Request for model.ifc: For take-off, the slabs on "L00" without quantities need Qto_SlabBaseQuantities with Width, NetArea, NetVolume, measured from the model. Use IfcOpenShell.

First a look at what the model holds.

```python
import ifcopenshell
import ifcopenshell.util.element
import ifcopenshell.util.unit

model = ifcopenshell.open("model.ifc")
print(model.schema)
for unit_type in ("LENGTHUNIT", "AREAUNIT", "VOLUMEUNIT"):
    print(unit_type, ifcopenshell.util.unit.calculate_unit_scale(model, unit_type))
storey = next(s for s in model.by_type("IfcBuildingStorey") if s.Name == "L00")
slabs = [e for e in ifcopenshell.util.element.get_decomposition(storey) if e.is_a("IfcSlab")]
for e in sorted(slabs, key=lambda e: e.id()):
    print(e.id(), e.is_a(), e.Name, list(ifcopenshell.util.element.get_psets(e, qtos_only=True)), sep=" | ")
```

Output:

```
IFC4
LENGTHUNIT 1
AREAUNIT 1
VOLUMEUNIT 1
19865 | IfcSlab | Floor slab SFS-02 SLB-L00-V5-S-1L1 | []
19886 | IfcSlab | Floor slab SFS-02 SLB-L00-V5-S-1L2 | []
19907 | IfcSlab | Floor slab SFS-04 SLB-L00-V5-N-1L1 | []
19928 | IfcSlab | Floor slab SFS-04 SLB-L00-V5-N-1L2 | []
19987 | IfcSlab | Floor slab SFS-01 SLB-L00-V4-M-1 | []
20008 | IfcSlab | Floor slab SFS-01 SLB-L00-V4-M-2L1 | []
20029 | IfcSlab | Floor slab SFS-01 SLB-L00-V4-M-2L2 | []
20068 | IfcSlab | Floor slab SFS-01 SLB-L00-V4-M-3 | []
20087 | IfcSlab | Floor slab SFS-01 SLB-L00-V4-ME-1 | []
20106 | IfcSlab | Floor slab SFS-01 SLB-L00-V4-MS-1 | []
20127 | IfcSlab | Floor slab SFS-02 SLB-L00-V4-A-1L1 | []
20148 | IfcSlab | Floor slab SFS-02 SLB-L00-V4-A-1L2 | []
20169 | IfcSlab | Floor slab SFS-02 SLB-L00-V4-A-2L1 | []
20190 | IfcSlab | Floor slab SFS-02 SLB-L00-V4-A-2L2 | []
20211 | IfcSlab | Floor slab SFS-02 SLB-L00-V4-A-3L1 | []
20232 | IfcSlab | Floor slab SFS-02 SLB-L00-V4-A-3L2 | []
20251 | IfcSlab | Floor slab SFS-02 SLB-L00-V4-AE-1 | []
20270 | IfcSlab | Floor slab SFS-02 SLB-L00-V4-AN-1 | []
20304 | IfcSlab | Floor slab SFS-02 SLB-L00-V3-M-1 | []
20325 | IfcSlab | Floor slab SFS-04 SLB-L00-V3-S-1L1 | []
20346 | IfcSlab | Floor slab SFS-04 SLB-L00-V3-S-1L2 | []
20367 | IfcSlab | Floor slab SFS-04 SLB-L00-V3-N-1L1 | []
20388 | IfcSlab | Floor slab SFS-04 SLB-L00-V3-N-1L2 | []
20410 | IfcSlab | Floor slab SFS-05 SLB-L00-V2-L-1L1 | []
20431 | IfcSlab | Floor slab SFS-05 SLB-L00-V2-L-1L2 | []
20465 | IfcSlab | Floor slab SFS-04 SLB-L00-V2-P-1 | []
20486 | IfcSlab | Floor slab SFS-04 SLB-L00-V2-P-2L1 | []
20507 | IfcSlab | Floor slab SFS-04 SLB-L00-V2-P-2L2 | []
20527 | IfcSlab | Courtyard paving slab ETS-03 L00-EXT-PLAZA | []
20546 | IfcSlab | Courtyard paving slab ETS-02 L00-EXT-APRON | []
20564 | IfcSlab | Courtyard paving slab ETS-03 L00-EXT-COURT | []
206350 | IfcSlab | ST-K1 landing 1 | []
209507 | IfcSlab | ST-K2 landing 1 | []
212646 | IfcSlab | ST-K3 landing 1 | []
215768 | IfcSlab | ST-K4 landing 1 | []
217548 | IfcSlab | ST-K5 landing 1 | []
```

```python
import ifcopenshell
import ifcopenshell.api.pset
import ifcopenshell.geom
import ifcopenshell.util.element
import ifcopenshell.util.shape
import ifcopenshell.util.unit

model = ifcopenshell.open("model.ifc")
unit_scale = ifcopenshell.util.unit.calculate_unit_scale(model)
area_scale = ifcopenshell.util.unit.calculate_unit_scale(model, "AREAUNIT")
volume_scale = ifcopenshell.util.unit.calculate_unit_scale(model, "VOLUMEUNIT")
settings = ifcopenshell.geom.settings()

storey = next(s for s in model.by_type("IfcBuildingStorey") if s.Name == "L00")
slabs = [e for e in ifcopenshell.util.element.get_decomposition(storey) if e.is_a("IfcSlab")]

for e in sorted(slabs, key=lambda e: e.id()):
    if ifcopenshell.util.element.get_psets(e, qtos_only=True, should_inherit=False):
        continue
    # Geometry comes back in metres, in the element's own axes.
    shape = ifcopenshell.geom.create_shape(settings, e)
    values = {
        "Width": ifcopenshell.util.shape.get_z(shape.geometry) / unit_scale,
        "NetArea": ifcopenshell.util.shape.get_footprint_area(shape.geometry) / area_scale,
        "NetVolume": ifcopenshell.util.shape.get_volume(shape.geometry) / volume_scale,
    }
    qto = ifcopenshell.api.pset.add_qto(model, product=e, name="Qto_SlabBaseQuantities")
    ifcopenshell.api.pset.edit_qto(model, qto=qto, properties=values)
    print(e.id(), {k: round(v, 3) for k, v in values.items()})

model.write("model_edited.ifc")
```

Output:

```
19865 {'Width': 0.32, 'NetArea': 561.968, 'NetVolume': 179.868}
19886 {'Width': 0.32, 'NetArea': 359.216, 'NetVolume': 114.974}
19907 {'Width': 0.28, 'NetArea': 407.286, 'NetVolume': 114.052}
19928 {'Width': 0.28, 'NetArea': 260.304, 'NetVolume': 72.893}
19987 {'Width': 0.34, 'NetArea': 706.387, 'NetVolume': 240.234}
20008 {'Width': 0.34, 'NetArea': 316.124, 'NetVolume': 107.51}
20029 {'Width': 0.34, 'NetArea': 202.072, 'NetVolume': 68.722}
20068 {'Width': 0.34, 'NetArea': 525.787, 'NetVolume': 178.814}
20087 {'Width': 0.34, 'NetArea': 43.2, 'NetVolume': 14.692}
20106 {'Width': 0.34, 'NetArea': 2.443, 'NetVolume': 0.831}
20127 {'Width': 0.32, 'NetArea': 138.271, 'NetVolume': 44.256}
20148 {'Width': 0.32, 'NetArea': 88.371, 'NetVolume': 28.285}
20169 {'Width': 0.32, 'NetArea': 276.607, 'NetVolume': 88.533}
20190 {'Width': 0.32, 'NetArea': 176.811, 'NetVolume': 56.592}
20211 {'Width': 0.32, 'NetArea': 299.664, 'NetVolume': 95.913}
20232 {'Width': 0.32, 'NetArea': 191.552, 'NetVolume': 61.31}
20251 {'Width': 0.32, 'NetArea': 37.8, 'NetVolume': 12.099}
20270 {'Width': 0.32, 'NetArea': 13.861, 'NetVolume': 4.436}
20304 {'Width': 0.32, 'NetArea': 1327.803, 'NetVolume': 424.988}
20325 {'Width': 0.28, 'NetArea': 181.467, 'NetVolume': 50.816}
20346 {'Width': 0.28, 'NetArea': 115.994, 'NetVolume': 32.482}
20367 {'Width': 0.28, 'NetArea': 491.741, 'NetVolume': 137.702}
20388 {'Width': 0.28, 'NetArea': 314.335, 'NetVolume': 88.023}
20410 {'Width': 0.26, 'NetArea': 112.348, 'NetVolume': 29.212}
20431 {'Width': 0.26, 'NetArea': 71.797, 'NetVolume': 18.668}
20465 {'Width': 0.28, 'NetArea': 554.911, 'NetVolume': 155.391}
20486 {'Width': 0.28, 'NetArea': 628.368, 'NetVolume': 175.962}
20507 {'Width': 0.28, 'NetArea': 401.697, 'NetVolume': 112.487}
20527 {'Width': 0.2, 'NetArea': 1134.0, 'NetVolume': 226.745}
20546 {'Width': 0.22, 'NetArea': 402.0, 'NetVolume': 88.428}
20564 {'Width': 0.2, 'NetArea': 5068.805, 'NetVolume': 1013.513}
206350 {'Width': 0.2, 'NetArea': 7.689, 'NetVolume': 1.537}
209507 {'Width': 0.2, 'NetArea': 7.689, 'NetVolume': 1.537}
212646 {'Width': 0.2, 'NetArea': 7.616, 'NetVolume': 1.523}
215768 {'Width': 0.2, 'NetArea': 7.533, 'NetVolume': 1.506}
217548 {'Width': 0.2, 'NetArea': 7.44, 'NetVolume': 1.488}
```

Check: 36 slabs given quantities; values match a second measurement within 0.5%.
